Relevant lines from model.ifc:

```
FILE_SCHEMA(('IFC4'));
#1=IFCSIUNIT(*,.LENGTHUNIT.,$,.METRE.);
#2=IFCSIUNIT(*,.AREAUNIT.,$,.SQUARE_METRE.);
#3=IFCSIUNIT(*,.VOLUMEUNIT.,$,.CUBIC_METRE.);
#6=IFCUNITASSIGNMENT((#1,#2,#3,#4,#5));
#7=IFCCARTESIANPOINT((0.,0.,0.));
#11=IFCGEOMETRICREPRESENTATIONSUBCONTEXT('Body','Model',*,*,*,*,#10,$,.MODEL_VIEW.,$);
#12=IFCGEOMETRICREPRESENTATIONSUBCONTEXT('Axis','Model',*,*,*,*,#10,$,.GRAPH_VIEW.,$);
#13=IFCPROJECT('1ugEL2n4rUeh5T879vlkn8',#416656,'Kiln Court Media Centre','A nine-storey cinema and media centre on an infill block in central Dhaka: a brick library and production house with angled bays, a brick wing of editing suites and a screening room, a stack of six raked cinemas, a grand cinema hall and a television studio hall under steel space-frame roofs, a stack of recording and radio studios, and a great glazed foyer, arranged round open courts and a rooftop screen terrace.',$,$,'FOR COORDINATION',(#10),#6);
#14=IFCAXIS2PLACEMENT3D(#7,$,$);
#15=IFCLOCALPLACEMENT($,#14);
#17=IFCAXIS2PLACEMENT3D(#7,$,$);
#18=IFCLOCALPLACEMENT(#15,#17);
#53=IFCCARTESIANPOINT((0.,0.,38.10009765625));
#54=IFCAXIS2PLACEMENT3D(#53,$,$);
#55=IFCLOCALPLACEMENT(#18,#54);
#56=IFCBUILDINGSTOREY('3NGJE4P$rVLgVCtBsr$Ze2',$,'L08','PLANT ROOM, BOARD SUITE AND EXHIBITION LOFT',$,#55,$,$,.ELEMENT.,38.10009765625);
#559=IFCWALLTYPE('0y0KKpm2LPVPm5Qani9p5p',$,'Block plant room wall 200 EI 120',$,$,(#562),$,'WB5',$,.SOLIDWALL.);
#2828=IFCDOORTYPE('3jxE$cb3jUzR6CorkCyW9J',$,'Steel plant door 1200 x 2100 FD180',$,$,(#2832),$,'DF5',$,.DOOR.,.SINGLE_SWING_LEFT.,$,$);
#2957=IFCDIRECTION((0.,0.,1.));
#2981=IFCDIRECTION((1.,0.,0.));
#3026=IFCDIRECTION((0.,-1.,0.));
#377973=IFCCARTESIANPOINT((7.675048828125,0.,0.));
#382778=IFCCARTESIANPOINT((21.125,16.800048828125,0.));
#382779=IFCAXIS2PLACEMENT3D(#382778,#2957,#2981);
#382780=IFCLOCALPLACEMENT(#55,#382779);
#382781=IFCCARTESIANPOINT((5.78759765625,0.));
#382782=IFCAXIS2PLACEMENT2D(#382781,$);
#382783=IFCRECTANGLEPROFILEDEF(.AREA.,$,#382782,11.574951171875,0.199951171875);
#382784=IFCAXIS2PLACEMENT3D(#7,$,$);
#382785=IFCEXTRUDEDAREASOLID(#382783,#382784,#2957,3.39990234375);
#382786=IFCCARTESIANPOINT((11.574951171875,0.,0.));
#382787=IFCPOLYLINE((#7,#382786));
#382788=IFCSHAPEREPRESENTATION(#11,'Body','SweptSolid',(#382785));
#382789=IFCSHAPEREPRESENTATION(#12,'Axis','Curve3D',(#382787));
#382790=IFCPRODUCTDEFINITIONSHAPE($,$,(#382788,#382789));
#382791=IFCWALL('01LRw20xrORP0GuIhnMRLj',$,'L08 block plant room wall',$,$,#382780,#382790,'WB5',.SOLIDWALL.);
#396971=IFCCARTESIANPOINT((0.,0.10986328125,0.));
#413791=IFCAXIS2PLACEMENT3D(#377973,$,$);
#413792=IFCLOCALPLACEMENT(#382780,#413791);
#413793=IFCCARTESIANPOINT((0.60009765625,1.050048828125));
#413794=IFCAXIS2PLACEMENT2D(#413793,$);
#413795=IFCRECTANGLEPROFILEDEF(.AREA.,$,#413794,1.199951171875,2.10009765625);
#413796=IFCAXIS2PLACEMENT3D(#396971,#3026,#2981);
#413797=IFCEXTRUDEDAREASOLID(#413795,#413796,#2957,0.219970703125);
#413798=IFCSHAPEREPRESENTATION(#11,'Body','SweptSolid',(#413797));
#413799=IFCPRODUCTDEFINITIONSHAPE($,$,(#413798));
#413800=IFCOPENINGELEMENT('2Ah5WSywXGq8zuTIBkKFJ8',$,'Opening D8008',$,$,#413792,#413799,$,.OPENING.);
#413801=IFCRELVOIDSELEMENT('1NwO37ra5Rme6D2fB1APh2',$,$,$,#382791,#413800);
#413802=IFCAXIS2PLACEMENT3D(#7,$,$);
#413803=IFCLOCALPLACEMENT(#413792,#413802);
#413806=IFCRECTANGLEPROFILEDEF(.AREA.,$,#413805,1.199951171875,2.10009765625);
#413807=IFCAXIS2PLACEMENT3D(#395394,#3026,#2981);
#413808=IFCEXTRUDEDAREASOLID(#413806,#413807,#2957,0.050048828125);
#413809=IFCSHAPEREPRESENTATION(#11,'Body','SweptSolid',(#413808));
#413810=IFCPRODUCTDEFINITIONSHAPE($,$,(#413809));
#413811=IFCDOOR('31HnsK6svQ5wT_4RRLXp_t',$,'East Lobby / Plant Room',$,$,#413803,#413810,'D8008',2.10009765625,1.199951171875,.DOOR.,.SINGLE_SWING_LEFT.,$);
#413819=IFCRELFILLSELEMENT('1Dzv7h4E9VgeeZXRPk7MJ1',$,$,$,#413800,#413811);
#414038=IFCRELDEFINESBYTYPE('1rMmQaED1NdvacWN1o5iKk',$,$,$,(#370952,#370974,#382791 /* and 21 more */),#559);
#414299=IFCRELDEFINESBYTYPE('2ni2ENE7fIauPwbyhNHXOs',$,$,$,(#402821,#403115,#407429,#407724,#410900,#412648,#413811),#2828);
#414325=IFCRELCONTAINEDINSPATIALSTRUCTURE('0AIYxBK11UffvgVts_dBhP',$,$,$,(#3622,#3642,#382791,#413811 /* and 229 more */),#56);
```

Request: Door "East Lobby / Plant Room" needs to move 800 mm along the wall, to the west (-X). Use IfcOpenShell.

```python
import ifcopenshell
import ifcopenshell.api.geometry
import ifcopenshell.util.placement
import ifcopenshell.util.unit

model = ifcopenshell.open("model.ifc")
unit_scale = ifcopenshell.util.unit.calculate_unit_scale(model)

door = model.by_id(413811)
opening = door.FillsVoids[0].RelatingOpeningElement
wall = opening.VoidsElements[0].RelatingBuildingElement

wall_matrix = ifcopenshell.util.placement.get_local_placement(wall.ObjectPlacement)
shift = wall_matrix[:3, 0] * -0.8 / unit_scale
before = ifcopenshell.util.placement.get_local_placement(door.ObjectPlacement)[:3, 3].copy()

# The door is placed relative to its opening, so it follows when the opening moves.
matrix = ifcopenshell.util.placement.get_local_placement(opening.ObjectPlacement)
matrix[:3, 3] += shift
ifcopenshell.api.geometry.edit_object_placement(
    model, product=opening, matrix=matrix, is_si=False, should_transform_children=True
)

after = ifcopenshell.util.placement.get_local_placement(door.ObjectPlacement)[:3, 3]
print("door moved by", (after - before).round(3) + 0.0)

model.write("model_rev.ifc")
```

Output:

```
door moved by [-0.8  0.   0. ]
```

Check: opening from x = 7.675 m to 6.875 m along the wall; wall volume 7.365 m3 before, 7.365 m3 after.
